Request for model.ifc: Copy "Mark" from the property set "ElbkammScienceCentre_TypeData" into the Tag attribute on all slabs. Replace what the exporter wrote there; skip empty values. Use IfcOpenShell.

First a look at what the model holds.

```python
import ifcopenshell
import ifcopenshell.util.element

model = ifcopenshell.open("model.ifc")
print(model.schema)
slabs = model.by_type("IfcSlab")
print(len(slabs), "slabs")
for e in slabs[:8]:
    source = ifcopenshell.util.element.get_pset(e, "ElbkammScienceCentre_TypeData", "Mark")
    target = e.Tag
    print(e.id(), repr(source), repr(target), sep=" | ")
```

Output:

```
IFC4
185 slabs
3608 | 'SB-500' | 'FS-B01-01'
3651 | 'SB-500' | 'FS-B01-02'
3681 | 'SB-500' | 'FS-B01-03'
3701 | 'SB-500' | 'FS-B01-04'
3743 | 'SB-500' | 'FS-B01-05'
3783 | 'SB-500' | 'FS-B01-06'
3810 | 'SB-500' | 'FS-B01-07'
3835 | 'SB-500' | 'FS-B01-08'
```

```python
import ifcopenshell
import ifcopenshell.util.element

model = ifcopenshell.open("model.ifc")

count = 0
for e in model.by_type("IfcSlab"):
    value = ifcopenshell.util.element.get_pset(e, "ElbkammScienceCentre_TypeData", "Mark")
    current = e.Tag
    if not value or not value.strip() or current == value:
        continue
    e.Tag = value
    count += 1

print(count, "slabs updated")

model.write("model_updated.ifc")
```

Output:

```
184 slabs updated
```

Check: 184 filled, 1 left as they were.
